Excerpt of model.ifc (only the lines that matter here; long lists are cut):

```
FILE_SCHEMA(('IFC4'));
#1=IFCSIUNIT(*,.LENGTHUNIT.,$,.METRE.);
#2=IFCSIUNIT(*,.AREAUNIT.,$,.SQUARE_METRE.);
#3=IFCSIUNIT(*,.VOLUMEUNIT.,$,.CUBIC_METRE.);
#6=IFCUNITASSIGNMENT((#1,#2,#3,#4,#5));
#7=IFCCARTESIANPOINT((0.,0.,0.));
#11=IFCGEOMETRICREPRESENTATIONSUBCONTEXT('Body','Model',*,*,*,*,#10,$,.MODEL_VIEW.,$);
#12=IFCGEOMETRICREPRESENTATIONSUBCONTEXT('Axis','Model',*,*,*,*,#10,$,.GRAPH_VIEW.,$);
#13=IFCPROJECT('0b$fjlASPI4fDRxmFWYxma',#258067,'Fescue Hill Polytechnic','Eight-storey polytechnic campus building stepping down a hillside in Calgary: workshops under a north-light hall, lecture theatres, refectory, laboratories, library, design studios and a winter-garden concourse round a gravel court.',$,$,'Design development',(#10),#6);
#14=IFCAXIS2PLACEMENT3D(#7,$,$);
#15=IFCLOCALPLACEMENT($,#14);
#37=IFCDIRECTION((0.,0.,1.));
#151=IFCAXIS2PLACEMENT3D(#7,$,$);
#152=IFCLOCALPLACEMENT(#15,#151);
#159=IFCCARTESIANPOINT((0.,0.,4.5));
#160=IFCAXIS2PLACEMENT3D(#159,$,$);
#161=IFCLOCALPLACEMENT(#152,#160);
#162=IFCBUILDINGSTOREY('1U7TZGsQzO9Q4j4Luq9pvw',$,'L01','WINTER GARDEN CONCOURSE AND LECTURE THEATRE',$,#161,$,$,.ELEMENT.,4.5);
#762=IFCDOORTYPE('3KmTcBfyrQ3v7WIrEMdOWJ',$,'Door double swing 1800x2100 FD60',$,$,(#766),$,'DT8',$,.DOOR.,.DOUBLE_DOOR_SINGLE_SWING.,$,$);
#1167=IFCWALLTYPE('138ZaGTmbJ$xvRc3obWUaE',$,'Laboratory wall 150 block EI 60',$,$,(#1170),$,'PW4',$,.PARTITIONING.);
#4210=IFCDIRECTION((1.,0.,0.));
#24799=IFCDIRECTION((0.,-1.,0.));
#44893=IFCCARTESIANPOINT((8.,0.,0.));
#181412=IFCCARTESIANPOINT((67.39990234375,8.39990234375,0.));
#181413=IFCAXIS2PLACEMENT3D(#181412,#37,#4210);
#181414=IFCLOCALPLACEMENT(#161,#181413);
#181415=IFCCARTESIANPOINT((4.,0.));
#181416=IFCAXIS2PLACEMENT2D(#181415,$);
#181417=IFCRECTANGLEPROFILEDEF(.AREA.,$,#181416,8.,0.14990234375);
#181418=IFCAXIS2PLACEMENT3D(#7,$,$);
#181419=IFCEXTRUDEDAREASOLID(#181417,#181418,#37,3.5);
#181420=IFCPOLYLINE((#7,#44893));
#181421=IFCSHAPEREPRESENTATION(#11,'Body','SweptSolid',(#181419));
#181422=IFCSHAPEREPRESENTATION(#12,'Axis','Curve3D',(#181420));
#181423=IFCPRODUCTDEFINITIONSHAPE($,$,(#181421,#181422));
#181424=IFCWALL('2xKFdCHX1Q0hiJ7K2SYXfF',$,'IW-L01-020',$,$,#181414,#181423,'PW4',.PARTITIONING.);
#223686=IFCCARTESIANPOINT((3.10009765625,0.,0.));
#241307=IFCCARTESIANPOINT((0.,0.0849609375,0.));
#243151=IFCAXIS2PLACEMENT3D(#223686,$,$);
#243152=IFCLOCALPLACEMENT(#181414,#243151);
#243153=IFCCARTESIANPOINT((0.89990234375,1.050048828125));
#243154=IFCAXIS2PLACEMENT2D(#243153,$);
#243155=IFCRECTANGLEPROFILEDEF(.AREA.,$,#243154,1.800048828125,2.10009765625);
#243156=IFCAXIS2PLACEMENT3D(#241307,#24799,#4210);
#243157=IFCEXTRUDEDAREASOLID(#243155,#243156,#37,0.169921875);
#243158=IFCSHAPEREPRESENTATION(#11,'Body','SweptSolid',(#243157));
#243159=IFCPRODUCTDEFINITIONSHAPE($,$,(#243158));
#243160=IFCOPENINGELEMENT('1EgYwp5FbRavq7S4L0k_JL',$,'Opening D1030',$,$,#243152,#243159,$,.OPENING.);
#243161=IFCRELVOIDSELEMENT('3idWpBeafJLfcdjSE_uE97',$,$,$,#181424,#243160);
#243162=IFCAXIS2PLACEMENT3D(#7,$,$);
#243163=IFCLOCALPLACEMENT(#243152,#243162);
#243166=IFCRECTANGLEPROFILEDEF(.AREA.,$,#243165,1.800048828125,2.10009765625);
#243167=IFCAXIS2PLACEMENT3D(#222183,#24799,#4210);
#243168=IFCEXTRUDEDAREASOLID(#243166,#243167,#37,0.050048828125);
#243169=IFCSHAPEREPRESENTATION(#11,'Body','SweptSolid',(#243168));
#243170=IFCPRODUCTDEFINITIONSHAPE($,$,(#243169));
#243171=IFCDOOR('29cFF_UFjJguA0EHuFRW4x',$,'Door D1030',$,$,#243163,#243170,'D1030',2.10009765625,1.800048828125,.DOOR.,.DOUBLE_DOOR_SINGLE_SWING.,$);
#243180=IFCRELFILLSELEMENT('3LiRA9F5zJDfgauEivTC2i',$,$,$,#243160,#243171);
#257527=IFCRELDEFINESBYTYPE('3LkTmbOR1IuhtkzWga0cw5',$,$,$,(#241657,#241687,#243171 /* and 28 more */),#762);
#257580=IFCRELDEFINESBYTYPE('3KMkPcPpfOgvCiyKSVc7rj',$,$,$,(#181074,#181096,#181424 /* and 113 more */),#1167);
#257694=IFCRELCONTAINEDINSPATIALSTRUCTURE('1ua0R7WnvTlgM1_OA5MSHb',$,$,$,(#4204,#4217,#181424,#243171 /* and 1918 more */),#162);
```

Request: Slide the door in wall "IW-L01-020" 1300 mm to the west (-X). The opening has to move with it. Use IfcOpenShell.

```python
import ifcopenshell
import ifcopenshell.api.geometry
import ifcopenshell.util.placement

model = ifcopenshell.open("model.ifc")

door = model.by_id(243171)
opening = door.FillsVoids[0].RelatingOpeningElement
wall = opening.VoidsElements[0].RelatingBuildingElement

wall_matrix = ifcopenshell.util.placement.get_local_placement(wall.ObjectPlacement)
shift = wall_matrix[:3, 0] * -1.3
before = ifcopenshell.util.placement.get_local_placement(door.ObjectPlacement)[:3, 3].copy()

# The door is placed relative to its opening, so it follows when the opening moves.
matrix = ifcopenshell.util.placement.get_local_placement(opening.ObjectPlacement)
matrix[:3, 3] += shift
ifcopenshell.api.geometry.edit_object_placement(
    model, product=opening, matrix=matrix, is_si=False, should_transform_children=True
)

after = ifcopenshell.util.placement.get_local_placement(door.ObjectPlacement)[:3, 3]
print("door moved by", (after - before).round(3) + 0.0)

model.write("model_rev.ifc")
```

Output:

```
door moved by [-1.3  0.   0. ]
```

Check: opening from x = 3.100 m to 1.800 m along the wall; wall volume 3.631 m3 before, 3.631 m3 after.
